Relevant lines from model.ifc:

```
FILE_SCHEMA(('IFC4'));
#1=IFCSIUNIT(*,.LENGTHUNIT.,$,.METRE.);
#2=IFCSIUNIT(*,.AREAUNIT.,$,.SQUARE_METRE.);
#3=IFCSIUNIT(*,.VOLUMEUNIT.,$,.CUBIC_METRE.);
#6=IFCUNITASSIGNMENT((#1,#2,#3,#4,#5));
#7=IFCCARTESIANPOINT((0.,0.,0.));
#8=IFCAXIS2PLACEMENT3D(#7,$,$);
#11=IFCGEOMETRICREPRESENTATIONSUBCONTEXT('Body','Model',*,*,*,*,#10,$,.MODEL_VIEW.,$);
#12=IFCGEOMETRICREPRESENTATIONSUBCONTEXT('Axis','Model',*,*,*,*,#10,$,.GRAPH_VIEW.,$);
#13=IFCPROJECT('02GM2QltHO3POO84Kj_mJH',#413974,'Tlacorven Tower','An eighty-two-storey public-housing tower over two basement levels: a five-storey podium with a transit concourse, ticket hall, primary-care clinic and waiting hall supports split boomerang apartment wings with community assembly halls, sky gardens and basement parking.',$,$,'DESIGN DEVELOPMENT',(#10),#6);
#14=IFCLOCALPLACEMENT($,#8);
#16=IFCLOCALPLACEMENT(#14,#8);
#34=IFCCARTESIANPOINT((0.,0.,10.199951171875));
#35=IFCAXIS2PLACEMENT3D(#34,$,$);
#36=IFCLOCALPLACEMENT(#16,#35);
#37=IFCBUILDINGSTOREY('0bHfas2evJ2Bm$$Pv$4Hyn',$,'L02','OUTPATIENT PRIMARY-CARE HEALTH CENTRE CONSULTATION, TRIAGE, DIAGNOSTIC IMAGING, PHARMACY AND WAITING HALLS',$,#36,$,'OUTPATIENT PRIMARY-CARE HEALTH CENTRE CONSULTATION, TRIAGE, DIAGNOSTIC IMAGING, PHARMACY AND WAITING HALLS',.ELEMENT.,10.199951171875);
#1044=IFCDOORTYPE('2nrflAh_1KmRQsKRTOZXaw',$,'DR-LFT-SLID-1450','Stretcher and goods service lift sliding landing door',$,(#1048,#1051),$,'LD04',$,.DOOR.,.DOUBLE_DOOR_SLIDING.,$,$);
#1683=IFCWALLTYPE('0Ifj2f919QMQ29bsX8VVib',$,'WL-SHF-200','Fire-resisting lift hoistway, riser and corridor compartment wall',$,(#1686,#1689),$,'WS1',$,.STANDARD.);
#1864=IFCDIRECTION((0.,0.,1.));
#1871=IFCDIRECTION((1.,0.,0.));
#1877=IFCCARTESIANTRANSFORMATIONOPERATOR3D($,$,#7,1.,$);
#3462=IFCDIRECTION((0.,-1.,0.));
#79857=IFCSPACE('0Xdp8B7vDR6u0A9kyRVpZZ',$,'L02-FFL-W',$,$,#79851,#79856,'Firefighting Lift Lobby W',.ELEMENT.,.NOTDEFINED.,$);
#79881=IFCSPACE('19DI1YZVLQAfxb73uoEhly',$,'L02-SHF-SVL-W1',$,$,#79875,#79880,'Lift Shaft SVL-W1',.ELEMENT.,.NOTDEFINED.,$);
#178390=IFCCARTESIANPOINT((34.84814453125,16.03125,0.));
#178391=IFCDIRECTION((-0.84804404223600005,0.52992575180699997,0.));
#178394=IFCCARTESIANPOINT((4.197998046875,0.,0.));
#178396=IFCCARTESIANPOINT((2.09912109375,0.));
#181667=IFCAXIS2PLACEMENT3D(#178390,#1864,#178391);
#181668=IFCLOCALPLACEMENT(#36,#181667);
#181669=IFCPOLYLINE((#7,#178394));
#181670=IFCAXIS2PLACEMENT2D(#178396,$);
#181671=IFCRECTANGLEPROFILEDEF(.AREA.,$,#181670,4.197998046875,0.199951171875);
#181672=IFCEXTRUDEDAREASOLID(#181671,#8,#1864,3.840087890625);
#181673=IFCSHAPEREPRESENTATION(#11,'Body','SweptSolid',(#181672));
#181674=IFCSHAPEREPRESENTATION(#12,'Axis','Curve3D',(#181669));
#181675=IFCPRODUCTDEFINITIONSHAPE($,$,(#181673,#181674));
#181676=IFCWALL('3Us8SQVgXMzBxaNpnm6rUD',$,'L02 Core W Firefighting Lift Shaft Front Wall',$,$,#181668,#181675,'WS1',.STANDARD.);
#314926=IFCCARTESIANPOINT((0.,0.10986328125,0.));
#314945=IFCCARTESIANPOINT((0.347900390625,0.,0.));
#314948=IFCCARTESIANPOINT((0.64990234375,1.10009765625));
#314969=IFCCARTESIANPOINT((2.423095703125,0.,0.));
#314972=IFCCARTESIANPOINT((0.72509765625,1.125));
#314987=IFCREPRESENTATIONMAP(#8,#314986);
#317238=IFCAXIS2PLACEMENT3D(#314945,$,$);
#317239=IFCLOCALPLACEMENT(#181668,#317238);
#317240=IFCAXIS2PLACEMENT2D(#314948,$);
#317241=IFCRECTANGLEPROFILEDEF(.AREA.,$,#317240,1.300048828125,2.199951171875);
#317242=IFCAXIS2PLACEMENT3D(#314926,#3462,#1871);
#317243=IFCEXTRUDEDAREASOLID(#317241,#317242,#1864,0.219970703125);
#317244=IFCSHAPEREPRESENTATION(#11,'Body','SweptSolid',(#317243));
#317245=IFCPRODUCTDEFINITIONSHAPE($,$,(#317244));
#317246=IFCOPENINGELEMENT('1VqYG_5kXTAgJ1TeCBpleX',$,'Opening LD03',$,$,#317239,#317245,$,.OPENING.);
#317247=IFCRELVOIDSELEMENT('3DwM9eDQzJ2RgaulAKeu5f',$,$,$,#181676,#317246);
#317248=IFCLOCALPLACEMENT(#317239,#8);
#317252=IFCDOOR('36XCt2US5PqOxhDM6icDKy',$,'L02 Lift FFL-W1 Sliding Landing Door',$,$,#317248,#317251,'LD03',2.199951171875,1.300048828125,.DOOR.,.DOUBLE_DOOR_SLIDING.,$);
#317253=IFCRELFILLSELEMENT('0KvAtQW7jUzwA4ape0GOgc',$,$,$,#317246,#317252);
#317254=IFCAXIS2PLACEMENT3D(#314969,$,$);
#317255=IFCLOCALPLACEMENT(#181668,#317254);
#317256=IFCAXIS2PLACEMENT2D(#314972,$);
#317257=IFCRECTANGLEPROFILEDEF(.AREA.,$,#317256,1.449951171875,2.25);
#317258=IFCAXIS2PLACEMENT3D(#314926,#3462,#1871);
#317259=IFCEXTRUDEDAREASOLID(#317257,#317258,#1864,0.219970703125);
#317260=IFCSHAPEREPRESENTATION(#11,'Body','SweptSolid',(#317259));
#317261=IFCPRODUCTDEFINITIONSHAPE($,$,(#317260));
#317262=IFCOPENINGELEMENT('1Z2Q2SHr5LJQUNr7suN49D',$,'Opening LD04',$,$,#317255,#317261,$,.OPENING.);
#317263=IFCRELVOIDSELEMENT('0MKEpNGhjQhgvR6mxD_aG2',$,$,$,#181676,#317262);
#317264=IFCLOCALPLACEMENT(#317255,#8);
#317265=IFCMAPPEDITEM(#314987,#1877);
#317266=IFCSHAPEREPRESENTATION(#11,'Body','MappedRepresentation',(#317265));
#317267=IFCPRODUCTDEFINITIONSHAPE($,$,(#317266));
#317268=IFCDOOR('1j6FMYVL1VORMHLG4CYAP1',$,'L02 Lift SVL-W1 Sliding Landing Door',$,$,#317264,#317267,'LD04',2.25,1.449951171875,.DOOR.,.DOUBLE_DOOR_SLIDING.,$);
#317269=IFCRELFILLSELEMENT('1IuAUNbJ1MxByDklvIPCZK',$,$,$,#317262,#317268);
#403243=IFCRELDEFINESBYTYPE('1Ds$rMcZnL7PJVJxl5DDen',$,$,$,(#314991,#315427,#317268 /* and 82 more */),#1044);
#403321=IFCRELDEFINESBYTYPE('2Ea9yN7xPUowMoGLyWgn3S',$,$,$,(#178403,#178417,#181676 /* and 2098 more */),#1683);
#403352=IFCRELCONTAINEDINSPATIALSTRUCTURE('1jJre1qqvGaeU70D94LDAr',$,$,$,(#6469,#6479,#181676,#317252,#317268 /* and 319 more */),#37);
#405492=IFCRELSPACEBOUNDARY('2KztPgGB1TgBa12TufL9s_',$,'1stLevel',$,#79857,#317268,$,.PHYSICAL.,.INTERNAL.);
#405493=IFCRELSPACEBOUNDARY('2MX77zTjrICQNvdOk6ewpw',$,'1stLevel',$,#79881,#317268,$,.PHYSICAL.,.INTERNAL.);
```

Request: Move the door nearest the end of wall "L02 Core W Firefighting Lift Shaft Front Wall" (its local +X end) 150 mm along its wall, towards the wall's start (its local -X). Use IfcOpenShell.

```python
import ifcopenshell
import ifcopenshell.api.geometry
import ifcopenshell.util.placement
import ifcopenshell.util.unit

model = ifcopenshell.open("model.ifc")
unit_scale = ifcopenshell.util.unit.calculate_unit_scale(model)

door = model.by_guid("1j6FMYVL1VORMHLG4CYAP1")
opening = door.FillsVoids[0].RelatingOpeningElement
wall = opening.VoidsElements[0].RelatingBuildingElement

wall_matrix = ifcopenshell.util.placement.get_local_placement(wall.ObjectPlacement)
shift = wall_matrix[:3, 0] * -0.15 / unit_scale
before = ifcopenshell.util.placement.get_local_placement(door.ObjectPlacement)[:3, 3].copy()

# The door is placed relative to its opening, so it follows when the opening moves.
matrix = ifcopenshell.util.placement.get_local_placement(opening.ObjectPlacement)
matrix[:3, 3] += shift
ifcopenshell.api.geometry.edit_object_placement(
    model, product=opening, matrix=matrix, is_si=False, should_transform_children=True
)

after = ifcopenshell.util.placement.get_local_placement(door.ObjectPlacement)[:3, 3]
print("door moved by", (after - before).round(3) + 0.0)

model.write("model_edited.ifc")
```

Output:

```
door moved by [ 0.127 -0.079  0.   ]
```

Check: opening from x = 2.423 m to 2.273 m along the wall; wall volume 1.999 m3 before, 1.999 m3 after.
